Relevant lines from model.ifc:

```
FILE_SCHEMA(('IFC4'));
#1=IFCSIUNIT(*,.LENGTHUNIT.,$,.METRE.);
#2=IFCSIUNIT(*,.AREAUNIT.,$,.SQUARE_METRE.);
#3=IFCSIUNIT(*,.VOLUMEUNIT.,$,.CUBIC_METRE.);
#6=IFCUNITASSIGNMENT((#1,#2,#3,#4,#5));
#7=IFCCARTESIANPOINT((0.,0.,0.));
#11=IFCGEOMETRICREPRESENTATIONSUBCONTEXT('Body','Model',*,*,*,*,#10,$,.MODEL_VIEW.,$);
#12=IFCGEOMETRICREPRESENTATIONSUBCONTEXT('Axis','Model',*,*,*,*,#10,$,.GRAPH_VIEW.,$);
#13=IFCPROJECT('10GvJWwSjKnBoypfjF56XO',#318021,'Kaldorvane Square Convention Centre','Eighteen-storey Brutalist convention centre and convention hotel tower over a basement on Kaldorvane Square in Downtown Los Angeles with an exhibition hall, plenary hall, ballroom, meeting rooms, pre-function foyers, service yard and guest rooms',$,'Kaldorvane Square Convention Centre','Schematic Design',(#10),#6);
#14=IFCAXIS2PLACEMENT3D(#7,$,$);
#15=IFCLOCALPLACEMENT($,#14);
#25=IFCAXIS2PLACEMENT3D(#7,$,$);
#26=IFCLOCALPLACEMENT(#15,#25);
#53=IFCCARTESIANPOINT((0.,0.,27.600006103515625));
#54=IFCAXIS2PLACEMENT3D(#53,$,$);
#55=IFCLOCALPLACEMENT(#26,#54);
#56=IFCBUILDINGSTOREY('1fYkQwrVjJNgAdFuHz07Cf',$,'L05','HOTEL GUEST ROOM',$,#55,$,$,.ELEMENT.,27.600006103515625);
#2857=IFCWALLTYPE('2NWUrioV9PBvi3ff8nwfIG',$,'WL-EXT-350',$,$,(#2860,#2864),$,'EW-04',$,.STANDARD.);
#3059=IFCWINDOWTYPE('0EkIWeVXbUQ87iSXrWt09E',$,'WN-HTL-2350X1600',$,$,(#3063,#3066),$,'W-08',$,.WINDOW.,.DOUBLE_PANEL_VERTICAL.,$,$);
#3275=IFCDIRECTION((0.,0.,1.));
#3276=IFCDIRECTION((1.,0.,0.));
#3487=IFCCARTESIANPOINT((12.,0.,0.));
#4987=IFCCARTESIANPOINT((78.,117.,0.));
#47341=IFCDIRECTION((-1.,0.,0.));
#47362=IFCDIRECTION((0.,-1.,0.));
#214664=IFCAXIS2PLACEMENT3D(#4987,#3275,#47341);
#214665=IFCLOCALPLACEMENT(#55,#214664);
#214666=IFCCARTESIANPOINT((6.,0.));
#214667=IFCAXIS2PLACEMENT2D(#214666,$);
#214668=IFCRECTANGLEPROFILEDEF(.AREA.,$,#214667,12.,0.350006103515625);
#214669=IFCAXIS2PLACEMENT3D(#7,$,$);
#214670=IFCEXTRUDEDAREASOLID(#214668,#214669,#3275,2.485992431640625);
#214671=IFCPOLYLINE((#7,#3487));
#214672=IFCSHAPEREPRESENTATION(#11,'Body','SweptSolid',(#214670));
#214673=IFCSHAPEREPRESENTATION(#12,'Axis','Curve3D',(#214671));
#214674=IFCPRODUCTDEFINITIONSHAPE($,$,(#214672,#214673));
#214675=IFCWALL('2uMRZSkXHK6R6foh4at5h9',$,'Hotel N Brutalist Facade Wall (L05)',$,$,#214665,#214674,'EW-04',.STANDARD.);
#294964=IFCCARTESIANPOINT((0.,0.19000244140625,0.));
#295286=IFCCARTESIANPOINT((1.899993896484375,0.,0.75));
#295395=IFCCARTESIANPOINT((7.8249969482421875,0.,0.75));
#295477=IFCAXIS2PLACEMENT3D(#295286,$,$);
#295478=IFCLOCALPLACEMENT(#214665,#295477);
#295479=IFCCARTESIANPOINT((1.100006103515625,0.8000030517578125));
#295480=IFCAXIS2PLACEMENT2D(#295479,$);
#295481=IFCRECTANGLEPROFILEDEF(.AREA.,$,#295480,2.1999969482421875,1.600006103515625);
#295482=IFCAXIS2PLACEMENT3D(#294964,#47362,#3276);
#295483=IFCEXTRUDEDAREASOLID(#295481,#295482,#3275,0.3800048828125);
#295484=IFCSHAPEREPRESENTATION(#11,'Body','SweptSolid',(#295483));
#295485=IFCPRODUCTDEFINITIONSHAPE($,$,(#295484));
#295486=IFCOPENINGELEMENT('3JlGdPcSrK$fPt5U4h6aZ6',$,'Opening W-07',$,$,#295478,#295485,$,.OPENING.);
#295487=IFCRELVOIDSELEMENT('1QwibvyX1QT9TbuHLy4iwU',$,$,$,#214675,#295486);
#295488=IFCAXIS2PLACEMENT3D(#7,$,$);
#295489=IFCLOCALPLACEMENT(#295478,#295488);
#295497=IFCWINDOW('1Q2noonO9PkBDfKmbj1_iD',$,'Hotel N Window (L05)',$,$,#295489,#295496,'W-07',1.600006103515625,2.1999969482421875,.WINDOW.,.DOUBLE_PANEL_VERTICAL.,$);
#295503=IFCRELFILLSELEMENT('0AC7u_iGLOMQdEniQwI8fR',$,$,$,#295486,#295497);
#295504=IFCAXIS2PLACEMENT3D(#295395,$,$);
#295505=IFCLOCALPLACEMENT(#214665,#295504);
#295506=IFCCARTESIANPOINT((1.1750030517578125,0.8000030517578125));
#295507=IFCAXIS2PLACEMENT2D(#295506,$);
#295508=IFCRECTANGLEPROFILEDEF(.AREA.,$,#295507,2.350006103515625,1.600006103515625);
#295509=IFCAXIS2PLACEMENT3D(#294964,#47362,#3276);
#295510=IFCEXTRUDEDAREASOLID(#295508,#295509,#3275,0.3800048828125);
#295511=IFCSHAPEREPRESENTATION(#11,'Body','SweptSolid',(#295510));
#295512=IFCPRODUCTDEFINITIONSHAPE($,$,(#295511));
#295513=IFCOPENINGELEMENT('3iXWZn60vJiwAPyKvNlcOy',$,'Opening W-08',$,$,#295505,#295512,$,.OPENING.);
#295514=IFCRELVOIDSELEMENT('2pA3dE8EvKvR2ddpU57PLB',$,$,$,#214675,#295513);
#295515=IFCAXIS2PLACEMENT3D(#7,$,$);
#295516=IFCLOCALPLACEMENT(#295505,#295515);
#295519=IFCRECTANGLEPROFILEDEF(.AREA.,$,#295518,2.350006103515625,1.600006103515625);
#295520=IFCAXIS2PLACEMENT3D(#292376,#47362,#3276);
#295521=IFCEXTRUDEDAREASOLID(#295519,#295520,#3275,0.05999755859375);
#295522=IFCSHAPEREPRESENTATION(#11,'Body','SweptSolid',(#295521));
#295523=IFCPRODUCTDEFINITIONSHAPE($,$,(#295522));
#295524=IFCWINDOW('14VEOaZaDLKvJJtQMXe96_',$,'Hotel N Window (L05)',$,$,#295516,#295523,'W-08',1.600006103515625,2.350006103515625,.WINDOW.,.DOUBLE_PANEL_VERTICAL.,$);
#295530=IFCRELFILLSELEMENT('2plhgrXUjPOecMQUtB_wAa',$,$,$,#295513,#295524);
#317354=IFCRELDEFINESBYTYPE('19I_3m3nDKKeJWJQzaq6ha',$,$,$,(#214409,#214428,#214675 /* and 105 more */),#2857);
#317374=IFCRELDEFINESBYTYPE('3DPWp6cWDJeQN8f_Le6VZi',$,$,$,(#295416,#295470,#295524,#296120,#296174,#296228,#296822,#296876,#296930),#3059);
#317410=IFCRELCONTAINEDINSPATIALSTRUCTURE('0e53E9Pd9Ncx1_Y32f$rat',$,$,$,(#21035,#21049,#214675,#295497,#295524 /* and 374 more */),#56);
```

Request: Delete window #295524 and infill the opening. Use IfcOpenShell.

```python
import ifcopenshell
import ifcopenshell.api.feature
import ifcopenshell.api.root
import ifcopenshell.geom
import ifcopenshell.util.shape

model = ifcopenshell.open("model.ifc")
settings = ifcopenshell.geom.settings()


def volume(element):
    """Net volume in cubic metres, openings subtracted."""
    shape = ifcopenshell.geom.create_shape(settings, element)
    return ifcopenshell.util.shape.get_volume(shape.geometry)


window = model.by_guid("14VEOaZaDLKvJJtQMXe96_")
opening = window.FillsVoids[0].RelatingOpeningElement
wall = opening.VoidsElements[0].RelatingBuildingElement
before = volume(wall)

ifcopenshell.api.root.remove_product(model, product=window)
ifcopenshell.api.feature.remove_feature(model, feature=opening)

after = volume(wall)

print(f"wall volume {before:.3f} -> {after:.3f} m3")

model.write("model_updated.ifc")
```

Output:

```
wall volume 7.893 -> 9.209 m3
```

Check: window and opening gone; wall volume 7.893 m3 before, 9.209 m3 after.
